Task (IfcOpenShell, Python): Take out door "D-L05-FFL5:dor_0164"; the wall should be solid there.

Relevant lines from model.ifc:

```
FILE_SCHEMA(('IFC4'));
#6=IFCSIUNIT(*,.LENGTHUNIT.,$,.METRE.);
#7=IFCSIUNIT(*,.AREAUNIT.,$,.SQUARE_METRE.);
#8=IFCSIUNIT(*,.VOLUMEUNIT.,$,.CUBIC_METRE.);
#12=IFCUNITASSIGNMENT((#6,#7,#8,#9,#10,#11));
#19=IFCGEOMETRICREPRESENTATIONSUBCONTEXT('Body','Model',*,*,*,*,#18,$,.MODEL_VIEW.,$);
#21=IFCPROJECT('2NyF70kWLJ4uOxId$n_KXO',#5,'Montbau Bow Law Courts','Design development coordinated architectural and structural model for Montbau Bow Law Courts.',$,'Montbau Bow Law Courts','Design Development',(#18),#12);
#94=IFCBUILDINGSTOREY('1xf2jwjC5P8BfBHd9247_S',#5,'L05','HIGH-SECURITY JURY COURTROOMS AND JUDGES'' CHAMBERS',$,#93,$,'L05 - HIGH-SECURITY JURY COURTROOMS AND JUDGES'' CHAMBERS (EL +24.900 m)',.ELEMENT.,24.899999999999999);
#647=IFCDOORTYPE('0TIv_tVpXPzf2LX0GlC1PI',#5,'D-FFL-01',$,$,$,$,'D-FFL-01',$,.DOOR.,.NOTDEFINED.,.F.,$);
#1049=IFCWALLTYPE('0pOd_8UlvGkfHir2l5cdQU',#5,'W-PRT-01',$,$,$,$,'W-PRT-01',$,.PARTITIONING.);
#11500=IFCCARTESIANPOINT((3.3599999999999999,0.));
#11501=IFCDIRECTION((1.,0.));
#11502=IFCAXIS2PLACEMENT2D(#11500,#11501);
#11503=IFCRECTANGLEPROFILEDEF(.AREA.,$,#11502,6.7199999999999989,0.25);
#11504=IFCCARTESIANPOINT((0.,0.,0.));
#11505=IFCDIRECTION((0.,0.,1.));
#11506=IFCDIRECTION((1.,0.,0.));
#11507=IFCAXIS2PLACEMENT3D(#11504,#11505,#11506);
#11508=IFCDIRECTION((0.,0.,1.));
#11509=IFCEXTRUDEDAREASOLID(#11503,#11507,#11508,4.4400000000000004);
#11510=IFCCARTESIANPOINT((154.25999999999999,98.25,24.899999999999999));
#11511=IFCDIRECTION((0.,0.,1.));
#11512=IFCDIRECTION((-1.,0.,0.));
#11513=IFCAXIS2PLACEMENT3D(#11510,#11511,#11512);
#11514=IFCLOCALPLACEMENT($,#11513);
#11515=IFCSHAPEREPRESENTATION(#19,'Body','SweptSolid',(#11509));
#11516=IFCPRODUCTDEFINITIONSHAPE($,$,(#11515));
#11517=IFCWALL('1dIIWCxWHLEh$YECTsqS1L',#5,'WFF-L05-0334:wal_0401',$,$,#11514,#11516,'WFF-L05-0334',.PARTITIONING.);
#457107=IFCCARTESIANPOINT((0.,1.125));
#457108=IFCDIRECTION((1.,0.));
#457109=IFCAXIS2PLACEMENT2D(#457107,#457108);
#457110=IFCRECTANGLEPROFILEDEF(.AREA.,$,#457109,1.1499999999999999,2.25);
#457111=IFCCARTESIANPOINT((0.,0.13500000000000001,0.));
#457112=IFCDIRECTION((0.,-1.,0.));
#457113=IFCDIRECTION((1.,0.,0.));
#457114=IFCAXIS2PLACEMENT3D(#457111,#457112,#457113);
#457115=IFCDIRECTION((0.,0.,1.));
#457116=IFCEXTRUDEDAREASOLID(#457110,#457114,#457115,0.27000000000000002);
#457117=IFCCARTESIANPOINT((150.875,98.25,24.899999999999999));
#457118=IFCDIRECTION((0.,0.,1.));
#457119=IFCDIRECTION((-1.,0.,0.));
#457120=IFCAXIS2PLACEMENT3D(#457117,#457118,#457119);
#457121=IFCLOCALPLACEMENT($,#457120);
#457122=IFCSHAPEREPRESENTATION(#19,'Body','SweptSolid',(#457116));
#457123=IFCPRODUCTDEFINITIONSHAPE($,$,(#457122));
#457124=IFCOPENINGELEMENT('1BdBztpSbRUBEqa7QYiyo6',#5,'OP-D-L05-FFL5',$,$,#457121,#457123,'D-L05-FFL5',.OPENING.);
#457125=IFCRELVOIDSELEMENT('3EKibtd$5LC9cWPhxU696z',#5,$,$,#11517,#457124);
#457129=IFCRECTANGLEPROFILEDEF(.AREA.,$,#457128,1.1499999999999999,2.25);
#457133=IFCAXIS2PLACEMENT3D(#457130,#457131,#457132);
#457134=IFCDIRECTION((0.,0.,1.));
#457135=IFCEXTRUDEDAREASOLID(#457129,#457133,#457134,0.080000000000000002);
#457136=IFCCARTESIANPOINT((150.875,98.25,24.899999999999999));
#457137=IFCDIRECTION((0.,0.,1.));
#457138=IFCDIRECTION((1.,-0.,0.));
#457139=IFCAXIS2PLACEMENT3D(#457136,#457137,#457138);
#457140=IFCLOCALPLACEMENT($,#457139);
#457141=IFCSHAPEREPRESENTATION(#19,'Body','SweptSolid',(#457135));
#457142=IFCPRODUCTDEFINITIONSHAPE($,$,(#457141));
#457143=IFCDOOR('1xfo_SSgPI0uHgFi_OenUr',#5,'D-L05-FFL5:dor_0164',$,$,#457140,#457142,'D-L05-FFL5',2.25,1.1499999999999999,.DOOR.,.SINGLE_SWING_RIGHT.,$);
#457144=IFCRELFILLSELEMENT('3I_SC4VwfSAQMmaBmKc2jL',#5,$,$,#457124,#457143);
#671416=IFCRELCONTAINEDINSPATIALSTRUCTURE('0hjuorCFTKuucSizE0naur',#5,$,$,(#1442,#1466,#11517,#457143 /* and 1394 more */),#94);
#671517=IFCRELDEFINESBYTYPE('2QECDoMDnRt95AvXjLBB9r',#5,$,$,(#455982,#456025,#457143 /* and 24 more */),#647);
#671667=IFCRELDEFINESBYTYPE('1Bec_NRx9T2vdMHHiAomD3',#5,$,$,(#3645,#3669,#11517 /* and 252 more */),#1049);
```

```python
import ifcopenshell
import ifcopenshell.api.feature
import ifcopenshell.api.root
import ifcopenshell.geom
import ifcopenshell.util.shape

model = ifcopenshell.open("model.ifc")
settings = ifcopenshell.geom.settings()


def volume(element):
    """Net volume in cubic metres, openings subtracted."""
    shape = ifcopenshell.geom.create_shape(settings, element)
    return ifcopenshell.util.shape.get_volume(shape.geometry)


door = model.by_guid("1xfo_SSgPI0uHgFi_OenUr")
opening = door.FillsVoids[0].RelatingOpeningElement
wall = opening.VoidsElements[0].RelatingBuildingElement
before = volume(wall)

ifcopenshell.api.root.remove_product(model, product=door)
ifcopenshell.api.feature.remove_feature(model, feature=opening)

after = volume(wall)

print(f"wall volume {before:.3f} -> {after:.3f} m3")

model.write("model_v2.ifc")
```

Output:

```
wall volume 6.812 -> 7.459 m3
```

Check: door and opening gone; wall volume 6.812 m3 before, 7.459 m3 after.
